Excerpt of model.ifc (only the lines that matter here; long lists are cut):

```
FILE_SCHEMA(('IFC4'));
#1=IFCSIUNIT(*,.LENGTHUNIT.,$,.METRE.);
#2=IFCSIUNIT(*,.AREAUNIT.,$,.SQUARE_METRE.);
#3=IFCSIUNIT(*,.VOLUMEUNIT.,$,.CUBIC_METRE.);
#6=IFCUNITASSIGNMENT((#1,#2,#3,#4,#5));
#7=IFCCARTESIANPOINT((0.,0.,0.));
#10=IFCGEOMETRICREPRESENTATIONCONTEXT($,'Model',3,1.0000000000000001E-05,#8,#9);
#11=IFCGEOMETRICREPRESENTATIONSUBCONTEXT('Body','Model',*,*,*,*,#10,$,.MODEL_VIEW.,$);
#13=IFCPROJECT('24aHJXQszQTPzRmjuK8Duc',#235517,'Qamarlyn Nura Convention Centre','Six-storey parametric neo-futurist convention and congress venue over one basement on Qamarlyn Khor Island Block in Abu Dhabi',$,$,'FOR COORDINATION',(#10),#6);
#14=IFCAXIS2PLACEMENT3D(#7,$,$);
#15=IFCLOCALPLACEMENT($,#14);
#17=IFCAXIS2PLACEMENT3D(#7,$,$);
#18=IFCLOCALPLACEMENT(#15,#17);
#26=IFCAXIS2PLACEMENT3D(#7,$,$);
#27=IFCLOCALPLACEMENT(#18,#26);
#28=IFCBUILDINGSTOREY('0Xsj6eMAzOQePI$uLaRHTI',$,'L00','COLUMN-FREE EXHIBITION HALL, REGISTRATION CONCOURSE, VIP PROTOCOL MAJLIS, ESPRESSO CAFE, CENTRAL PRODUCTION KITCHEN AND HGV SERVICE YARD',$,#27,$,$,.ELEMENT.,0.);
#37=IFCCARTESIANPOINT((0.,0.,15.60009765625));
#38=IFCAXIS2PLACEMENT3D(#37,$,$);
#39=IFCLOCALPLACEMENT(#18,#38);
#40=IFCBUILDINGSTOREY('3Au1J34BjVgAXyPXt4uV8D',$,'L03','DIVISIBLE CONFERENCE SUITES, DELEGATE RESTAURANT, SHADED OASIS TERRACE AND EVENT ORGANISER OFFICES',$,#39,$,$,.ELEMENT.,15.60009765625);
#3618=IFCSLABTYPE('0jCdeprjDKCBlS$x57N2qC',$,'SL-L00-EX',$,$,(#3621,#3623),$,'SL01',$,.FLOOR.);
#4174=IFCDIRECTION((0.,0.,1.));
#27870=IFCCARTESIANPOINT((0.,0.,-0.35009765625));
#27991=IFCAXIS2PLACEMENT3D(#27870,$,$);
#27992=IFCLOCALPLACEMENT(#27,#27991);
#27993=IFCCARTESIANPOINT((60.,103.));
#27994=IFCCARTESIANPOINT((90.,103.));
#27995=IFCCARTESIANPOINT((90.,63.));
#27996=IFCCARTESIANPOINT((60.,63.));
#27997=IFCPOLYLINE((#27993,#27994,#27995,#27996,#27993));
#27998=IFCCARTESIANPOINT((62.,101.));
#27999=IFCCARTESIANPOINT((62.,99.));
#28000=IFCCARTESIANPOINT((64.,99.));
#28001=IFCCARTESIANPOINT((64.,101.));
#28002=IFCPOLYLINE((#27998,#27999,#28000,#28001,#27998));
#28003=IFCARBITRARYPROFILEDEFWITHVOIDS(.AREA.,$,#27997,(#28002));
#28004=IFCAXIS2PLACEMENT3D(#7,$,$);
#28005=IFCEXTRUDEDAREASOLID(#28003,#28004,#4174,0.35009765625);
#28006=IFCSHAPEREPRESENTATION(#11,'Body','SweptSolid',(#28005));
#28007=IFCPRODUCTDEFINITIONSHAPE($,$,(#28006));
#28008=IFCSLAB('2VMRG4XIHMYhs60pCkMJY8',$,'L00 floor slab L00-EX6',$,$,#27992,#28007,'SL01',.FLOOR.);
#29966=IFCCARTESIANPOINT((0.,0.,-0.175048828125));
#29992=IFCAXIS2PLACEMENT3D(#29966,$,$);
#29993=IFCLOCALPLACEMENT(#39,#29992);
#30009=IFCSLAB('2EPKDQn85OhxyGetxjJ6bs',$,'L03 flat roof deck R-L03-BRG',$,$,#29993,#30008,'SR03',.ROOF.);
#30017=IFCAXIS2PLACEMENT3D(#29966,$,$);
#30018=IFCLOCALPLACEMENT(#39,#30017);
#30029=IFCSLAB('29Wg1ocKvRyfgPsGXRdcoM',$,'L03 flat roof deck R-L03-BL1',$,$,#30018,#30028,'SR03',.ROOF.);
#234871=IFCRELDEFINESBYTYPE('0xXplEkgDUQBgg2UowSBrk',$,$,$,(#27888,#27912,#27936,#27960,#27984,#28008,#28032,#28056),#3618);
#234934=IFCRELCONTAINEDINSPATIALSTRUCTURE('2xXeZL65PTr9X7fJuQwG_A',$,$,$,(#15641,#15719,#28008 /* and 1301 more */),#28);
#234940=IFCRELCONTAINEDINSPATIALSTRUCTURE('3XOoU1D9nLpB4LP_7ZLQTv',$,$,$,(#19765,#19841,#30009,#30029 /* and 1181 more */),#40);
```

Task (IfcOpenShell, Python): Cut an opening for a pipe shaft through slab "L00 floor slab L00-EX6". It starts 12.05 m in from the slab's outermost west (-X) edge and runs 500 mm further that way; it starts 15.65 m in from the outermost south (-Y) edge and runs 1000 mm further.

```python
import numpy as np
import ifcopenshell
import ifcopenshell.api.feature
import ifcopenshell.api.geometry
import ifcopenshell.api.root
import ifcopenshell.geom
import ifcopenshell.util.placement
import ifcopenshell.util.representation
import ifcopenshell.util.shape
import ifcopenshell.util.unit

model = ifcopenshell.open("model.ifc")
unit_scale = ifcopenshell.util.unit.calculate_unit_scale(model)
settings = ifcopenshell.geom.settings()


def volume(element):
    """Net volume in cubic metres, openings subtracted."""
    shape = ifcopenshell.geom.create_shape(settings, element)
    return ifcopenshell.util.shape.get_volume(shape.geometry)


slab = model.by_guid("2VMRG4XIHMYhs60pCkMJY8")
before = volume(slab)

# Extent in the slab's own axes, in metres. The edges named are its -X and -Y sides.
slab_shape = ifcopenshell.geom.create_shape(settings, slab)
vertices = ifcopenshell.util.shape.get_vertices(slab_shape.geometry)
x_min, y_min, bottom = vertices.min(axis=0)
top = vertices[:, 2].max()

opening = ifcopenshell.api.root.create_entity(model, ifc_class="IfcOpeningElement", name="Pipe shaft opening", predefined_type="OPENING")
context = ifcopenshell.util.representation.get_context(model, "Model", "Body", "MODEL_VIEW")
width, depth = 0.5, 1
outline = [(0.0, 0.0), (width, 0.0), (width, depth), (0.0, depth), (0.0, 0.0)]
# Overshoot both faces by 50 mm so the cut is clean.
shape = ifcopenshell.api.geometry.add_slab_representation(
    model, context=context, depth=top - bottom + 0.1, polyline=outline
)
ifcopenshell.api.geometry.assign_representation(model, product=opening, representation=shape)

matrix = ifcopenshell.util.placement.get_local_placement(slab.ObjectPlacement)
matrix[:, 3] = matrix @ np.append(np.array([x_min + 12.05, y_min + 15.65, bottom - 0.05]) / unit_scale, 1.0)
ifcopenshell.api.geometry.edit_object_placement(model, product=opening, matrix=matrix, is_si=False)
ifcopenshell.api.feature.add_feature(model, feature=opening, element=slab)

after = volume(slab)

print(f"slab volume {before:.3f} -> {after:.3f} m3")

model.write("model-out.ifc")
```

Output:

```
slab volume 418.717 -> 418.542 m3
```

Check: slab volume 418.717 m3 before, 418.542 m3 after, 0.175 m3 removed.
